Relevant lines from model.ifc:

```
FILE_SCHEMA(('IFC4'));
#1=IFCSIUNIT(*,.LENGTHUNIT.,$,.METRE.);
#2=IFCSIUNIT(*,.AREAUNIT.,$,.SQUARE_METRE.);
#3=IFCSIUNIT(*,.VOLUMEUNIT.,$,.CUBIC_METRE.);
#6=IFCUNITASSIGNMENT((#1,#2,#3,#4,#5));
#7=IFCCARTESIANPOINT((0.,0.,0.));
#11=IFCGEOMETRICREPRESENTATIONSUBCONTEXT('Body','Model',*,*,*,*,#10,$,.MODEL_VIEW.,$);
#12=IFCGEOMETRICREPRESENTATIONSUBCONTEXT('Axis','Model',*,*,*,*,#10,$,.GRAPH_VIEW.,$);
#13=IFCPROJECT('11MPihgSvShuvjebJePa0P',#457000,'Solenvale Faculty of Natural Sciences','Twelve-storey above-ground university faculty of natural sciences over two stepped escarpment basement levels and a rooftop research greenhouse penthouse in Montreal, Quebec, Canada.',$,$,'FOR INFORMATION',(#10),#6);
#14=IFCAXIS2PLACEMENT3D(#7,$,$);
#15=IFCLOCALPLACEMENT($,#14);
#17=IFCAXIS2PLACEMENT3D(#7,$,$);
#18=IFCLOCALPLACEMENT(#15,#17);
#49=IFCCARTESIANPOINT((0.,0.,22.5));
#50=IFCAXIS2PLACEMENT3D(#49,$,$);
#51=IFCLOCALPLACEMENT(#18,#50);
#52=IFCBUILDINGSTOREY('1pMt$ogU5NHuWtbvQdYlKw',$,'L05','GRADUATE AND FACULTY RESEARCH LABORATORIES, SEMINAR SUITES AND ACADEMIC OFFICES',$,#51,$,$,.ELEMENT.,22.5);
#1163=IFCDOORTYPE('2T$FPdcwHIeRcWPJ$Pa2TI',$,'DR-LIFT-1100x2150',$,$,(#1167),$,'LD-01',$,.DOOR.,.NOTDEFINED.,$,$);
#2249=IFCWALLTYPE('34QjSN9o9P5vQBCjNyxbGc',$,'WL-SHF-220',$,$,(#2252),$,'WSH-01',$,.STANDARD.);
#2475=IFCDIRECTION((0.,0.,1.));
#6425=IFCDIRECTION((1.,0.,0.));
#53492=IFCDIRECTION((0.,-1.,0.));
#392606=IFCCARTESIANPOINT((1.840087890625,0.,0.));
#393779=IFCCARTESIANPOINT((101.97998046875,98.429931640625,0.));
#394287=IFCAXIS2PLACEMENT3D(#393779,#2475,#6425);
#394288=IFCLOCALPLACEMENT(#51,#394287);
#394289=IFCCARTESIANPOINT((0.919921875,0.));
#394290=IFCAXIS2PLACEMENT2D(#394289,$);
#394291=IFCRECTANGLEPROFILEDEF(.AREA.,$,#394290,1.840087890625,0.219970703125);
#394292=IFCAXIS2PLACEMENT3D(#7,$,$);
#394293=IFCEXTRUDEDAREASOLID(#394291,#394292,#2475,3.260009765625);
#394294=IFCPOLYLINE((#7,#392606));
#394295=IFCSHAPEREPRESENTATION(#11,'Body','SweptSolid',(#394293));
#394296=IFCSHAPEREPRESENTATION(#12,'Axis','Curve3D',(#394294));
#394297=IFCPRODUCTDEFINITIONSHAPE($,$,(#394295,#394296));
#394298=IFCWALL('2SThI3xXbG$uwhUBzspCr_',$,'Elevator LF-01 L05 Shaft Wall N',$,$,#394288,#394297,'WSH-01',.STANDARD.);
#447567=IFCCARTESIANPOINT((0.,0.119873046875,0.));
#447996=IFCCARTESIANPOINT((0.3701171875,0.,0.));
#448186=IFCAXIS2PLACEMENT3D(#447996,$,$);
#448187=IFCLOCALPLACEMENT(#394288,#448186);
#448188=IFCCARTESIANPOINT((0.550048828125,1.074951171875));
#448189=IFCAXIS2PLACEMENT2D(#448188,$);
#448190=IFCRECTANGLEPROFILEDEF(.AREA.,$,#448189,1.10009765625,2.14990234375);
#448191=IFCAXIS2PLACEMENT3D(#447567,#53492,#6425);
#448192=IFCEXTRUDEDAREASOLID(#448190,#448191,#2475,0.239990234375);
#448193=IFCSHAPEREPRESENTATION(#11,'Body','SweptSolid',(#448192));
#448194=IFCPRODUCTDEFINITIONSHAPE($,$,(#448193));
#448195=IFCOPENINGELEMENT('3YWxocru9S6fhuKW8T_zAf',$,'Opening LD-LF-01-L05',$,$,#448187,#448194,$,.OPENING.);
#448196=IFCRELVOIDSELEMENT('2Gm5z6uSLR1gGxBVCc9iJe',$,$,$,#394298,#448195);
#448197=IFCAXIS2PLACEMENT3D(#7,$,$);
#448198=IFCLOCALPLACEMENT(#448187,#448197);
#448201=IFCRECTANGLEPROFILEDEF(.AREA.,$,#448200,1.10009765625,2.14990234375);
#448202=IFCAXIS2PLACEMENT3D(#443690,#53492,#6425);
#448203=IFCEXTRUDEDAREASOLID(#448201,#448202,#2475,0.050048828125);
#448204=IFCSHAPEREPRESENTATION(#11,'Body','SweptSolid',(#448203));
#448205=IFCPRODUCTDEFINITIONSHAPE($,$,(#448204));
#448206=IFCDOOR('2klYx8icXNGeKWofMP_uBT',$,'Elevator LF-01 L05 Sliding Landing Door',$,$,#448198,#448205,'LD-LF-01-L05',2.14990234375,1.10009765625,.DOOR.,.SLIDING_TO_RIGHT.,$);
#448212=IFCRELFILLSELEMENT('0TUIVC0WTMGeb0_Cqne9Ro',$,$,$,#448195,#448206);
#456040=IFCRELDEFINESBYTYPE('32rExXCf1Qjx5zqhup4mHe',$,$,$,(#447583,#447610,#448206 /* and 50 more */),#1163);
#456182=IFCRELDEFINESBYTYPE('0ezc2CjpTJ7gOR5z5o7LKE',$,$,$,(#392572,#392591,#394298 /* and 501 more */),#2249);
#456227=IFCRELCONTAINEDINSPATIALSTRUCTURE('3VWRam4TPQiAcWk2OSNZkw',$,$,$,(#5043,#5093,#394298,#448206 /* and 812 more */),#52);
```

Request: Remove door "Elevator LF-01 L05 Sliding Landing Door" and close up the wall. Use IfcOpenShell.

```python
import ifcopenshell
import ifcopenshell.api.feature
import ifcopenshell.api.root
import ifcopenshell.geom
import ifcopenshell.util.shape

model = ifcopenshell.open("model.ifc")
settings = ifcopenshell.geom.settings()


def volume(element):
    """Net volume in cubic metres, openings subtracted."""
    shape = ifcopenshell.geom.create_shape(settings, element)
    return ifcopenshell.util.shape.get_volume(shape.geometry)


door = model.by_id(448206)
opening = door.FillsVoids[0].RelatingOpeningElement
wall = opening.VoidsElements[0].RelatingBuildingElement
before = volume(wall)

ifcopenshell.api.root.remove_product(model, product=door)
ifcopenshell.api.feature.remove_feature(model, feature=opening)

after = volume(wall)

print(f"wall volume {before:.3f} -> {after:.3f} m3")

model.write("model_v2.ifc")
```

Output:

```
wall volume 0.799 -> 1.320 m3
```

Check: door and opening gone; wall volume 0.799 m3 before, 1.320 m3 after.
